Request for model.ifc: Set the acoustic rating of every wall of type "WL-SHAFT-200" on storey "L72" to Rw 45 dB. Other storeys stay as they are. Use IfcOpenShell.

First a look at what the model holds.

```python
import ifcopenshell
import ifcopenshell.util.element

model = ifcopenshell.open("model.ifc")
print(model.schema)
storey = next(s for s in model.by_type("IfcBuildingStorey") if s.Name == "L72")
walls = [e for e in ifcopenshell.util.element.get_decomposition(storey) if e.is_a("IfcWall")]
seen = {}
for e in walls:
    element_type = ifcopenshell.util.element.get_type(e)
    key = (element_type.Name if element_type != e and element_type else None, ifcopenshell.util.element.get_pset(e, "Pset_WallCommon", "AcousticRating"))
    seen[key] = seen.get(key, 0) + 1
for (name, value), count in sorted(seen.items(), key=str):
    print(count, "x", name, "|", value)
```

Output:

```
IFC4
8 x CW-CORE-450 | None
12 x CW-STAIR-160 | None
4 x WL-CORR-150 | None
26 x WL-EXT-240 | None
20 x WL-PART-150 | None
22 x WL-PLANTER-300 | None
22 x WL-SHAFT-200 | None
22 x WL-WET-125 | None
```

```python
import ifcopenshell
import ifcopenshell.api.pset
import ifcopenshell.util.element

model = ifcopenshell.open("model.ifc")

storey = next(s for s in model.by_type("IfcBuildingStorey") if s.Name == "L72")
walls = [e for e in ifcopenshell.util.element.get_decomposition(storey) if e.is_a("IfcWall")]

count = 0
for e in walls:
    element_type = ifcopenshell.util.element.get_type(e)
    if element_type in (None, e) or element_type.Name != "WL-SHAFT-200":
        continue
    found = ifcopenshell.util.element.get_pset(e, "Pset_WallCommon", should_inherit=False)
    if found:
        pset = model.by_id(found["id"])
        if len(ifcopenshell.util.element.get_elements_by_pset(pset)) > 1:
            pset = ifcopenshell.api.pset.unshare_pset(model, products=[e], pset=pset)[0]
    else:
        pset = ifcopenshell.api.pset.add_pset(model, product=e, name="Pset_WallCommon")
    ifcopenshell.api.pset.edit_pset(model, pset=pset, properties={"AcousticRating": "Rw 45 dB"})
    count += 1

print(count, "walls updated")

model.write("model-out.ifc")
```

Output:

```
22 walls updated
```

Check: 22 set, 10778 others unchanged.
